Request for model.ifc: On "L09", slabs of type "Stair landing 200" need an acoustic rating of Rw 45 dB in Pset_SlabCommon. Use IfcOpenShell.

First a look at what the model holds.

```python
import ifcopenshell
import ifcopenshell.util.element

model = ifcopenshell.open("model.ifc")
print(model.schema)
storey = next(s for s in model.by_type("IfcBuildingStorey") if s.Name == "L09")
slabs = [e for e in ifcopenshell.util.element.get_decomposition(storey) if e.is_a("IfcSlab")]
seen = {}
for e in slabs:
    element_type = ifcopenshell.util.element.get_type(e)
    key = (element_type.Name if element_type != e and element_type else None, ifcopenshell.util.element.get_pset(e, "Pset_SlabCommon", "AcousticRating"))
    seen[key] = seen.get(key, 0) + 1
for (name, value), count in sorted(seen.items(), key=str):
    print(count, "x", name, "|", value)
```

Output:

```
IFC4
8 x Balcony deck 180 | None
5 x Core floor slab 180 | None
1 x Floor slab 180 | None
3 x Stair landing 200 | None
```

```python
import ifcopenshell
import ifcopenshell.api.pset
import ifcopenshell.util.element

model = ifcopenshell.open("model.ifc")

storey = next(s for s in model.by_type("IfcBuildingStorey") if s.Name == "L09")
slabs = [e for e in ifcopenshell.util.element.get_decomposition(storey) if e.is_a("IfcSlab")]

count = 0
for e in slabs:
    element_type = ifcopenshell.util.element.get_type(e)
    if element_type in (None, e) or element_type.Name != "Stair landing 200":
        continue
    found = ifcopenshell.util.element.get_pset(e, "Pset_SlabCommon", should_inherit=False)
    if found:
        pset = model.by_id(found["id"])
        if len(ifcopenshell.util.element.get_elements_by_pset(pset)) > 1:
            pset = ifcopenshell.api.pset.unshare_pset(model, products=[e], pset=pset)[0]
    else:
        pset = ifcopenshell.api.pset.add_pset(model, product=e, name="Pset_SlabCommon")
    ifcopenshell.api.pset.edit_pset(model, pset=pset, properties={"AcousticRating": "Rw 45 dB"})
    count += 1

print(count, "slabs updated")

model.write("model-out.ifc")
```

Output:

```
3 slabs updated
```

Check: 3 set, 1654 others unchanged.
